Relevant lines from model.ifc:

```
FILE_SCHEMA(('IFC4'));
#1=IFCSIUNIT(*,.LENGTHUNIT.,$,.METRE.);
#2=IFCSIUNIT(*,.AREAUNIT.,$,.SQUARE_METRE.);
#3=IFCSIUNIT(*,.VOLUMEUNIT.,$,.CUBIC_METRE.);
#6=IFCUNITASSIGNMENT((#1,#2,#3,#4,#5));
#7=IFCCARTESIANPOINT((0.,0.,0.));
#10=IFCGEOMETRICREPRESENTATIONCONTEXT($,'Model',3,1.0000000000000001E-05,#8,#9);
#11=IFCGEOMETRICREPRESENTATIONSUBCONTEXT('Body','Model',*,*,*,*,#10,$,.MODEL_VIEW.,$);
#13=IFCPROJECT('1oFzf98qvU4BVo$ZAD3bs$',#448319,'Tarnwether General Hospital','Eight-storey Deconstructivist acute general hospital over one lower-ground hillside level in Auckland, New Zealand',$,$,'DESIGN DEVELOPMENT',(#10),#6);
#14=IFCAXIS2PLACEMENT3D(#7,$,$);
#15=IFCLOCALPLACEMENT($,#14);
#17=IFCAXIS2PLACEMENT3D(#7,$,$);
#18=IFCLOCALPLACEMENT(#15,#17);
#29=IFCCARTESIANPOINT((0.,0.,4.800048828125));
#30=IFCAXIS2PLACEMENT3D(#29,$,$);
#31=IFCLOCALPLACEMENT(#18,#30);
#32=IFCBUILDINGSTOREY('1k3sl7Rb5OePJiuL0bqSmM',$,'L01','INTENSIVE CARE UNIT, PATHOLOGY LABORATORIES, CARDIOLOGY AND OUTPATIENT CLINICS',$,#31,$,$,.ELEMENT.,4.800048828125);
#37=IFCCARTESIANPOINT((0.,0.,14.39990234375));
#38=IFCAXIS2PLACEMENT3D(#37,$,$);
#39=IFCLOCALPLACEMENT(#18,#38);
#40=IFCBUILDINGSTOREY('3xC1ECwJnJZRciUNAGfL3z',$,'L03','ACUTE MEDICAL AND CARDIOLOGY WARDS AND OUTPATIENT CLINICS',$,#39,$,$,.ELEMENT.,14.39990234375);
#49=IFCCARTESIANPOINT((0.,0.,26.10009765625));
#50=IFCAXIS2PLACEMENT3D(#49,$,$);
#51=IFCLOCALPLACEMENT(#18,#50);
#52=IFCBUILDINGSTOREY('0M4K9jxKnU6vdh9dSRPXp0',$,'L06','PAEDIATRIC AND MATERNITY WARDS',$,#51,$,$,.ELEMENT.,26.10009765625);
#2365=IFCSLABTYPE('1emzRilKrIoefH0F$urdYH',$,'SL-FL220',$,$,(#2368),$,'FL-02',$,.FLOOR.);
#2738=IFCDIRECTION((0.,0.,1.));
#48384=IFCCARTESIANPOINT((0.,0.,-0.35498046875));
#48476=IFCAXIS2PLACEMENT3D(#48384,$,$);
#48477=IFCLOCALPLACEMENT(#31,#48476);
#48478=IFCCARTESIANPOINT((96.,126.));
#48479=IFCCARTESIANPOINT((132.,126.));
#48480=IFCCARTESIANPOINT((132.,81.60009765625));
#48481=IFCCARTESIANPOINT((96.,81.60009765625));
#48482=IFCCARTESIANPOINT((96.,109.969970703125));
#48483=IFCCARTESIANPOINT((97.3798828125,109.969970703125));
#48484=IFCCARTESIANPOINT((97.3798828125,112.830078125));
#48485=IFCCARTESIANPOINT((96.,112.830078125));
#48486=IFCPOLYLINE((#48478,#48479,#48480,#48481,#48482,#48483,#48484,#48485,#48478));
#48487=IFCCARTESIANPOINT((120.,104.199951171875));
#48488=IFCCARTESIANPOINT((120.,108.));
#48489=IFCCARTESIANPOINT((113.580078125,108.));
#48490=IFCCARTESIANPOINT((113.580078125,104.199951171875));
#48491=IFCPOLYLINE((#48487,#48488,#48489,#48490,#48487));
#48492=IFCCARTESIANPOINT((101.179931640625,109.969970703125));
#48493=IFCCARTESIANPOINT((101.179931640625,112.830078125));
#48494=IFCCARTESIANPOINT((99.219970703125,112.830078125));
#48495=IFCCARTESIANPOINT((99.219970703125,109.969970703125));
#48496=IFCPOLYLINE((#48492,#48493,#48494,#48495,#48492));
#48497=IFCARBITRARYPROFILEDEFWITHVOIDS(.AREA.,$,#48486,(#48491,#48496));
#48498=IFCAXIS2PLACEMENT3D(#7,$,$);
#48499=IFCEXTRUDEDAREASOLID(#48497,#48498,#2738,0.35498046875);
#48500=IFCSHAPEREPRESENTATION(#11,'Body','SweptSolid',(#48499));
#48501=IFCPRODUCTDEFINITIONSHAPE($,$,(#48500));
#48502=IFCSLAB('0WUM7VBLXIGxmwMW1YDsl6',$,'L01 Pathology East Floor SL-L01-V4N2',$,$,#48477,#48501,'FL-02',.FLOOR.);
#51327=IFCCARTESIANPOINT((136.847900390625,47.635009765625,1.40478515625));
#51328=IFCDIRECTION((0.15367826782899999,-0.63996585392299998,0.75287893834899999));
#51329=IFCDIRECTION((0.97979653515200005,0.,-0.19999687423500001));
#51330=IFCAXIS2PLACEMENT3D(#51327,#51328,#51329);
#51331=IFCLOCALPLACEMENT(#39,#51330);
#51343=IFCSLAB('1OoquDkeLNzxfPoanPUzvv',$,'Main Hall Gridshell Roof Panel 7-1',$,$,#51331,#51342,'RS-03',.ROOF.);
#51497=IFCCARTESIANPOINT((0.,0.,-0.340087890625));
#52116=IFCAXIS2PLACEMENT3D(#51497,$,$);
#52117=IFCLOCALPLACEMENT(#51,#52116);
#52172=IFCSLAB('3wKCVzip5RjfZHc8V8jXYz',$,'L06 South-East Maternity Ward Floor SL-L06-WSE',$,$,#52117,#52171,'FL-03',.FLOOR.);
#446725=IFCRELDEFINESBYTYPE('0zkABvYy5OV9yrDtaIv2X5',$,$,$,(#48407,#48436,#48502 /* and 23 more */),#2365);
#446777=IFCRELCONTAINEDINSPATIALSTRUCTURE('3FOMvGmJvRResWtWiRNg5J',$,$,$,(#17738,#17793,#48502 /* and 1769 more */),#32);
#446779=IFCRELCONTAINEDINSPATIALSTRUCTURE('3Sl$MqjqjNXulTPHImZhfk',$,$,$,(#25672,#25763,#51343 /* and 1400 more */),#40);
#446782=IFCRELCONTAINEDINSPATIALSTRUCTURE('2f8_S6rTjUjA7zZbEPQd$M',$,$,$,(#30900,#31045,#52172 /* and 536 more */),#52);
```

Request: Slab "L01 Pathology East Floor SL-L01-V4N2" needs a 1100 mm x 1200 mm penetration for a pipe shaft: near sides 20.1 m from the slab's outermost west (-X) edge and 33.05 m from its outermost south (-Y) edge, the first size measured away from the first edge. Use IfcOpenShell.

```python
import numpy as np
import ifcopenshell
import ifcopenshell.api.feature
import ifcopenshell.api.geometry
import ifcopenshell.api.root
import ifcopenshell.geom
import ifcopenshell.util.placement
import ifcopenshell.util.representation
import ifcopenshell.util.shape
import ifcopenshell.util.unit

model = ifcopenshell.open("model.ifc")
unit_scale = ifcopenshell.util.unit.calculate_unit_scale(model)
settings = ifcopenshell.geom.settings()


def volume(element):
    """Net volume in cubic metres, openings subtracted."""
    shape = ifcopenshell.geom.create_shape(settings, element)
    return ifcopenshell.util.shape.get_volume(shape.geometry)


slab = model.by_guid("0WUM7VBLXIGxmwMW1YDsl6")
before = volume(slab)

# Extent in the slab's own axes, in metres. The edges named are its -X and -Y sides.
slab_shape = ifcopenshell.geom.create_shape(settings, slab)
vertices = ifcopenshell.util.shape.get_vertices(slab_shape.geometry)
x_min, y_min, bottom = vertices.min(axis=0)
top = vertices[:, 2].max()

opening = ifcopenshell.api.root.create_entity(model, ifc_class="IfcOpeningElement", name="Pipe shaft opening", predefined_type="OPENING")
context = ifcopenshell.util.representation.get_context(model, "Model", "Body", "MODEL_VIEW")
width, depth = 1.1, 1.2
outline = [(0.0, 0.0), (width, 0.0), (width, depth), (0.0, depth), (0.0, 0.0)]
# Overshoot both faces by 50 mm so the cut is clean.
shape = ifcopenshell.api.geometry.add_slab_representation(
    model, context=context, depth=top - bottom + 0.1, polyline=outline
)
ifcopenshell.api.geometry.assign_representation(model, product=opening, representation=shape)

matrix = ifcopenshell.util.placement.get_local_placement(slab.ObjectPlacement)
matrix[:, 3] = matrix @ np.append(np.array([x_min + 20.1, y_min + 33.05, bottom - 0.05]) / unit_scale, 1.0)
ifcopenshell.api.geometry.edit_object_placement(model, product=opening, matrix=matrix, is_si=False)
ifcopenshell.api.feature.add_feature(model, feature=opening, element=slab)

after = volume(slab)

print(f"slab volume {before:.3f} -> {after:.3f} m3")

model.write("model-out.ifc")
```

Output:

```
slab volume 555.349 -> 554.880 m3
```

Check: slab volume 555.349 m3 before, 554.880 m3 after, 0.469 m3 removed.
